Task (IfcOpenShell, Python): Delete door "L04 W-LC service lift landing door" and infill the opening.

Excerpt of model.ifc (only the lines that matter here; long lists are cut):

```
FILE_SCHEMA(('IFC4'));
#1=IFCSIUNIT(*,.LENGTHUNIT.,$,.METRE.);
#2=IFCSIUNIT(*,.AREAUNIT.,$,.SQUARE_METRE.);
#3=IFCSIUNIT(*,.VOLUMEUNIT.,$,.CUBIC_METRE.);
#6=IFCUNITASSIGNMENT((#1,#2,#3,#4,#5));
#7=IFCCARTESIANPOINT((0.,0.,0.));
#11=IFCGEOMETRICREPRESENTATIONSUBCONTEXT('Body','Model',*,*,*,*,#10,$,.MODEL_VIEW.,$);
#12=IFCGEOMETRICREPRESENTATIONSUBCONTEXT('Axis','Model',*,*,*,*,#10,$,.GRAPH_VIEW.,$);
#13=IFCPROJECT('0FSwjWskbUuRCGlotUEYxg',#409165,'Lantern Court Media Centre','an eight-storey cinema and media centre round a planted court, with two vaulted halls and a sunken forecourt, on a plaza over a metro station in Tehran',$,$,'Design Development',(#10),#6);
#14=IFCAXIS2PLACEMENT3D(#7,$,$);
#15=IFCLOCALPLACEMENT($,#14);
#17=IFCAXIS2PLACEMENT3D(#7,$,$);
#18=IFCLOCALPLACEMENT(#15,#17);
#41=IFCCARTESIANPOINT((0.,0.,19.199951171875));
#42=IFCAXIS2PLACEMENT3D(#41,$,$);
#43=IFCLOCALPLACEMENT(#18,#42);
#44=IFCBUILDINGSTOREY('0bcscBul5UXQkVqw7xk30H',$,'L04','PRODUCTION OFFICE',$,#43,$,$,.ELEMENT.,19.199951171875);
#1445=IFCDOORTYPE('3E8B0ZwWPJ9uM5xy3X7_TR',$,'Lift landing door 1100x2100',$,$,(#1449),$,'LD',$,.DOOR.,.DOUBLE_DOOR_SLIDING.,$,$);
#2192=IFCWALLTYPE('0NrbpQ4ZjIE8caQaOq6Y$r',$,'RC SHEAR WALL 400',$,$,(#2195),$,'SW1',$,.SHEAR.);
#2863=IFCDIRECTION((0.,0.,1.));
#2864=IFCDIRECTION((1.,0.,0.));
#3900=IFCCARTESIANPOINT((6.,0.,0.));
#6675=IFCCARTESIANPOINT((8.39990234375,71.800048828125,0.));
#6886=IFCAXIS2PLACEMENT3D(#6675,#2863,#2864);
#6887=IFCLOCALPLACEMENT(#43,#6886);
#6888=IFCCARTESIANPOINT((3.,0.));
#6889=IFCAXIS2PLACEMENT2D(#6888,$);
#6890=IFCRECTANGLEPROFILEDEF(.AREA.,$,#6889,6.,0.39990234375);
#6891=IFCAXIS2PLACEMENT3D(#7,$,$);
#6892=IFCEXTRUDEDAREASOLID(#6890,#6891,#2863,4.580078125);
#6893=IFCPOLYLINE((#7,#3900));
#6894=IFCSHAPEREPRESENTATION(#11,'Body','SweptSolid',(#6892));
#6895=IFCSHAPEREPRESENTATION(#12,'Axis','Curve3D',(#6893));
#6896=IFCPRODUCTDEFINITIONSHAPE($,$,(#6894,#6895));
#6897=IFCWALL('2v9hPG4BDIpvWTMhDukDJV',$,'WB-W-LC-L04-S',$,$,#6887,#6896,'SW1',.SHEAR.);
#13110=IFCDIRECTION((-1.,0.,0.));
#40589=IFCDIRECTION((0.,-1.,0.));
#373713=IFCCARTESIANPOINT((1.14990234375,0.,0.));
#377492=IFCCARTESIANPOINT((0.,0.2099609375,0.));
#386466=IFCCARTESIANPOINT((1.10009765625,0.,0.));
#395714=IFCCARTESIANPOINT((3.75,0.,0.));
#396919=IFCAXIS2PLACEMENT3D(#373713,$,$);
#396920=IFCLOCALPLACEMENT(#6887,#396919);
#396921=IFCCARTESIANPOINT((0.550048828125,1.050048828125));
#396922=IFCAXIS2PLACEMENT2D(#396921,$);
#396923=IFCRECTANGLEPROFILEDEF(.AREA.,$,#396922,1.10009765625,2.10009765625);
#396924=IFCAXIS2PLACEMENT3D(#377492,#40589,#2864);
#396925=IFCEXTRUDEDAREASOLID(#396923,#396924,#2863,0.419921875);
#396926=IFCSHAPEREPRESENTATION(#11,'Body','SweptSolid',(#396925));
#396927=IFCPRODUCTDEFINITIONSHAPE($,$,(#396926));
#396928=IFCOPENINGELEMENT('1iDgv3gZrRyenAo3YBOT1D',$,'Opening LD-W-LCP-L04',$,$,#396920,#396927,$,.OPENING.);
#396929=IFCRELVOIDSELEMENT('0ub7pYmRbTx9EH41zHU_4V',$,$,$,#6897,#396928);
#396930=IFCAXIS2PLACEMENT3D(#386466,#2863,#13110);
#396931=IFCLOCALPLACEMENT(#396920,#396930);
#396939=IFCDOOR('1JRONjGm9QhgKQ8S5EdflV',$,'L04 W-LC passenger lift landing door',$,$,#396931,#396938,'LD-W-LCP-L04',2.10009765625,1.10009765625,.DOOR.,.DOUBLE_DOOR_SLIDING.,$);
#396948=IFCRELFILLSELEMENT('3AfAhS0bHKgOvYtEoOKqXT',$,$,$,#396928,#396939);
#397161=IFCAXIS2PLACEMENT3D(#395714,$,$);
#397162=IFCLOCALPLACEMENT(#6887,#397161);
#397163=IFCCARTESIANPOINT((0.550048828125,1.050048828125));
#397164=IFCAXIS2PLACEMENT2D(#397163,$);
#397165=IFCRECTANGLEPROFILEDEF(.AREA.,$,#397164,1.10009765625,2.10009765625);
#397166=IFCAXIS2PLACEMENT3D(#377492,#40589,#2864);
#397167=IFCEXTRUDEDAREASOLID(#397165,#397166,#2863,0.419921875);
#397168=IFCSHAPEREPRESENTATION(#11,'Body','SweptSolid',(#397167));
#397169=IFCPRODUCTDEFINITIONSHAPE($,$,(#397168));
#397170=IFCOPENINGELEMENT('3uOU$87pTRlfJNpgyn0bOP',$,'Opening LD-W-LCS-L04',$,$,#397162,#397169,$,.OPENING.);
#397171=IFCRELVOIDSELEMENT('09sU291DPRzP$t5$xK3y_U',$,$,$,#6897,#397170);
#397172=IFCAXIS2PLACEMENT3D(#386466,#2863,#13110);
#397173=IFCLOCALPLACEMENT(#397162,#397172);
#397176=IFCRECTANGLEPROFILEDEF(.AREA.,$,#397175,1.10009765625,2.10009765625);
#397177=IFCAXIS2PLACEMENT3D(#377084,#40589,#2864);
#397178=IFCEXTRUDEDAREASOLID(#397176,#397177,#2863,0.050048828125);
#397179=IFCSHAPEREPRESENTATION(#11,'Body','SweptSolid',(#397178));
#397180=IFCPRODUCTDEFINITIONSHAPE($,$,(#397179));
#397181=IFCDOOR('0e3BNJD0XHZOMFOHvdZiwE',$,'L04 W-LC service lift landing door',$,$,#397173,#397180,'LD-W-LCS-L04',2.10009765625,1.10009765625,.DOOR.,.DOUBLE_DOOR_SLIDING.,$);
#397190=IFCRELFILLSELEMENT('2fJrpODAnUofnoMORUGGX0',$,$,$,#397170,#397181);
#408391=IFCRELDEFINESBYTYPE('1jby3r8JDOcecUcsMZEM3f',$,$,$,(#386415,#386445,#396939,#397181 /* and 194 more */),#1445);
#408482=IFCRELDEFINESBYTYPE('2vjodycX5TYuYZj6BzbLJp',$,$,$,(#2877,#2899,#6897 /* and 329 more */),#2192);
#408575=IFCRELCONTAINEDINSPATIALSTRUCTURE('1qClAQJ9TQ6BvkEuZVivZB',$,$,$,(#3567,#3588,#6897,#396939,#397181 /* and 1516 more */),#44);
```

```python
import ifcopenshell
import ifcopenshell.api.feature
import ifcopenshell.api.root
import ifcopenshell.geom
import ifcopenshell.util.shape

model = ifcopenshell.open("model.ifc")
settings = ifcopenshell.geom.settings()


def volume(element):
    """Net volume in cubic metres, openings subtracted."""
    shape = ifcopenshell.geom.create_shape(settings, element)
    return ifcopenshell.util.shape.get_volume(shape.geometry)


door = model.by_guid("0e3BNJD0XHZOMFOHvdZiwE")
opening = door.FillsVoids[0].RelatingOpeningElement
wall = opening.VoidsElements[0].RelatingBuildingElement
before = volume(wall)

ifcopenshell.api.root.remove_product(model, product=door)
ifcopenshell.api.feature.remove_feature(model, feature=opening)

after = volume(wall)

print(f"wall volume {before:.3f} -> {after:.3f} m3")

model.write("model-out.ifc")
```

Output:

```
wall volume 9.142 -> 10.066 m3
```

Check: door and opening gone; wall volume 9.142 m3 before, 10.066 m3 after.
